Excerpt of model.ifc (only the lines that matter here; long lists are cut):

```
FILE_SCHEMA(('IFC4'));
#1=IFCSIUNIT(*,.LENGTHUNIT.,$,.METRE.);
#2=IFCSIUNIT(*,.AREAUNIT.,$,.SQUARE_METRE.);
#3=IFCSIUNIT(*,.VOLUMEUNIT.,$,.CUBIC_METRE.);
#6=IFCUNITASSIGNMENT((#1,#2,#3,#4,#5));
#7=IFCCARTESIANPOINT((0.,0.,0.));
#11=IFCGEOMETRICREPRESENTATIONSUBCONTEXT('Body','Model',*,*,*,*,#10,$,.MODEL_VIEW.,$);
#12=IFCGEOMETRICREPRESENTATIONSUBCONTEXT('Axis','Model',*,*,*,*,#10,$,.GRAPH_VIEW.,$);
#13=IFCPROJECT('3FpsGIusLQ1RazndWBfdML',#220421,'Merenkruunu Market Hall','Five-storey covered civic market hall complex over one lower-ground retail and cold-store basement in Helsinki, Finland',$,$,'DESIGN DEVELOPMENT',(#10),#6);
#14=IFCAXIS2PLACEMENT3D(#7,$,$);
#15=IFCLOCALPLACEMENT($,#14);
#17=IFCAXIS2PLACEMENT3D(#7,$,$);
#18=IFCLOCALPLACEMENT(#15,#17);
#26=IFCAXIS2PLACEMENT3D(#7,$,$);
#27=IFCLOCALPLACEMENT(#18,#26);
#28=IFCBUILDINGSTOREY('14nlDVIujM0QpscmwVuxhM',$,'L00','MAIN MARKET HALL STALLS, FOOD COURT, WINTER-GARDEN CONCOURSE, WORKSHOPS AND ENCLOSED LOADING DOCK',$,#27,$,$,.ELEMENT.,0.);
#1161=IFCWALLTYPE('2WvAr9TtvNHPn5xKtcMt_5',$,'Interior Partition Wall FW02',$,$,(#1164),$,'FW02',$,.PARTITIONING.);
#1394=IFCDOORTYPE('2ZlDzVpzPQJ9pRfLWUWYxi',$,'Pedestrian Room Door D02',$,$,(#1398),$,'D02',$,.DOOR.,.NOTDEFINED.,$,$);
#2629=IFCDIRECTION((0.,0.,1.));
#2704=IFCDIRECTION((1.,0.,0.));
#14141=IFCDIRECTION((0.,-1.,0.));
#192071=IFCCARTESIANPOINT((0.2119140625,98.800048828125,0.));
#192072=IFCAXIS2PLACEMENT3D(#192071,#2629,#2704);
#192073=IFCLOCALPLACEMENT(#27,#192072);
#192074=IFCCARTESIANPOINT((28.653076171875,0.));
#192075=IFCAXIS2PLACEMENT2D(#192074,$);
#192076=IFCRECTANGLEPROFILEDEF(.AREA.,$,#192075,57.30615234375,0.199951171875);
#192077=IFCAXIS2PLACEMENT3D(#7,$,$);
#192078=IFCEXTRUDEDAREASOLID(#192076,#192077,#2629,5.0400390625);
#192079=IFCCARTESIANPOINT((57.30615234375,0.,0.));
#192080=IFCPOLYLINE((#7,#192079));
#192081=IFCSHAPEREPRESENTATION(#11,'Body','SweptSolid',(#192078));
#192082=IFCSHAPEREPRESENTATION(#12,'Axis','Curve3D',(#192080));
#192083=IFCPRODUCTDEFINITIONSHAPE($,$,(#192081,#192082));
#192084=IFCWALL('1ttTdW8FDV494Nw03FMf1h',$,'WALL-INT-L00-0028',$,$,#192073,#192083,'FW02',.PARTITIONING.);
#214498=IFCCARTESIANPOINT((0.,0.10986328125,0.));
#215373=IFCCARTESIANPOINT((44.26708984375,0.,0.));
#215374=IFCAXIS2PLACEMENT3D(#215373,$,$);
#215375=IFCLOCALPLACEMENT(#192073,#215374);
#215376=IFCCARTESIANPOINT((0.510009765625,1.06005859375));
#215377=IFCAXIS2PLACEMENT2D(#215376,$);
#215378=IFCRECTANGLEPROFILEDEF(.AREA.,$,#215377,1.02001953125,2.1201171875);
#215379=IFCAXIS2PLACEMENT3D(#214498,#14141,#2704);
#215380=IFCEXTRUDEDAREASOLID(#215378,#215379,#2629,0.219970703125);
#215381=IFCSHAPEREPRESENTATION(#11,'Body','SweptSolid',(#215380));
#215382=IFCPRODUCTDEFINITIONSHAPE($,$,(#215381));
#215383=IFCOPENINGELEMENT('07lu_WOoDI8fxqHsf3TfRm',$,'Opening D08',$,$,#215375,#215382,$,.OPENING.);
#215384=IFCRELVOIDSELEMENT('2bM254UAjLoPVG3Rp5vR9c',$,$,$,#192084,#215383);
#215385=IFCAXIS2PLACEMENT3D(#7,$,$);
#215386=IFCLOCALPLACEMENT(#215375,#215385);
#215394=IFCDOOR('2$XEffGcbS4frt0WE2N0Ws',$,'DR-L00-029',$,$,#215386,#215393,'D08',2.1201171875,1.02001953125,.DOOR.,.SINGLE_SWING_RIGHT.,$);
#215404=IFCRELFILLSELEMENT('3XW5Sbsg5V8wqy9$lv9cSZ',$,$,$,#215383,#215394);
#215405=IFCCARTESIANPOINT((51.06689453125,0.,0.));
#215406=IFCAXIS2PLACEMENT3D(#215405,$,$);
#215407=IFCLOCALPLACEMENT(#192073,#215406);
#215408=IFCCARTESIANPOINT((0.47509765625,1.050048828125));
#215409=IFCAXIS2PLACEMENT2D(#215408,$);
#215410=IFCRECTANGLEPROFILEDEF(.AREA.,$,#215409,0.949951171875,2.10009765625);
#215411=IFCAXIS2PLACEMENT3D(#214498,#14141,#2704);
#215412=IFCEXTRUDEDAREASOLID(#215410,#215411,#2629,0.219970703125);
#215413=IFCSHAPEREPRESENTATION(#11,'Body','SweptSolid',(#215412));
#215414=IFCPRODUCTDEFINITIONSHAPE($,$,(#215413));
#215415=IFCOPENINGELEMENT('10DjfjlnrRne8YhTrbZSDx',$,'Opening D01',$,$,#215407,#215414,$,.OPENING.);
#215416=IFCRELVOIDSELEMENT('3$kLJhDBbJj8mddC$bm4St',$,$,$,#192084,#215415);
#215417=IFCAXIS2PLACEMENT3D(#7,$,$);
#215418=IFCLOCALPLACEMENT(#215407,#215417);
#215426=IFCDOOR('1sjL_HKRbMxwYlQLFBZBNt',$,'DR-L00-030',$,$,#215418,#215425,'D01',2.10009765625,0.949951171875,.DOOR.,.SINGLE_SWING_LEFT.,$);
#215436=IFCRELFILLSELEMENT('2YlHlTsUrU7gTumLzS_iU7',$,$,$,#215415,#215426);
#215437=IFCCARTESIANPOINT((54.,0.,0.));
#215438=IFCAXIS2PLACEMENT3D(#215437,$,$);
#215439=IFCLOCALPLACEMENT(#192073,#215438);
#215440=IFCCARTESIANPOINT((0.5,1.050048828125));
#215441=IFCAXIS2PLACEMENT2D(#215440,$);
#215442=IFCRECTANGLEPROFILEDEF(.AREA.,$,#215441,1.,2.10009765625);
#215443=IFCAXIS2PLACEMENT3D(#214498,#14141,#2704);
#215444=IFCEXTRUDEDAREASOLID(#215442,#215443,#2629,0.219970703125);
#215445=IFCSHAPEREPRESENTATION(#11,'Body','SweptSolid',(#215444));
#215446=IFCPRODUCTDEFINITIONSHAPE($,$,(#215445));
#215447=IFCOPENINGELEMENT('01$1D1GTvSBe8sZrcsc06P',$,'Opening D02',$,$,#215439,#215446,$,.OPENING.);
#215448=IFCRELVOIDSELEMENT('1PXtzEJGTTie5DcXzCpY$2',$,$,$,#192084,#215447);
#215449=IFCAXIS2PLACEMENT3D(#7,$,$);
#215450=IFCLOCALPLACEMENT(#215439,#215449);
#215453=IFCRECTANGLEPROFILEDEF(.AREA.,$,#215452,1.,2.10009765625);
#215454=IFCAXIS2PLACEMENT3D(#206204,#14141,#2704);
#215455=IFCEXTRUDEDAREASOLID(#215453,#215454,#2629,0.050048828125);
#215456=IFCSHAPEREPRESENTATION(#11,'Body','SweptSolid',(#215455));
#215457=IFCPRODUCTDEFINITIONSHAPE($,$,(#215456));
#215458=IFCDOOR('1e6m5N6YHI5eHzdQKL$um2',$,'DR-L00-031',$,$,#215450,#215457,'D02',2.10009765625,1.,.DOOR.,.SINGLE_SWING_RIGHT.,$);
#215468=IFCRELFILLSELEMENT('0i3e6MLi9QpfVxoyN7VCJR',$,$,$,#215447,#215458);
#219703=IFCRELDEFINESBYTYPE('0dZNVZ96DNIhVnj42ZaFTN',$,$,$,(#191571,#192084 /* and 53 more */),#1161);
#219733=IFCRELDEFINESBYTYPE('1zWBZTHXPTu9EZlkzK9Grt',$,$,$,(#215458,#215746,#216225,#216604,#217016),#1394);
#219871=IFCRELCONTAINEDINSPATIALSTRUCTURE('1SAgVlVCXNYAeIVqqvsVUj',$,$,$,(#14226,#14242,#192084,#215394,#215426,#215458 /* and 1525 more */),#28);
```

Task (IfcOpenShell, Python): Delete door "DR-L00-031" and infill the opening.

```python
import ifcopenshell
import ifcopenshell.api.feature
import ifcopenshell.api.root
import ifcopenshell.geom
import ifcopenshell.util.shape

model = ifcopenshell.open("model.ifc")
settings = ifcopenshell.geom.settings()


def volume(element):
    """Net volume in cubic metres, openings subtracted."""
    shape = ifcopenshell.geom.create_shape(settings, element)
    return ifcopenshell.util.shape.get_volume(shape.geometry)


door = model.by_guid("1e6m5N6YHI5eHzdQKL$um2")
opening = door.FillsVoids[0].RelatingOpeningElement
wall = opening.VoidsElements[0].RelatingBuildingElement
before = volume(wall)

ifcopenshell.api.root.remove_product(model, product=door)
ifcopenshell.api.feature.remove_feature(model, feature=opening)

after = volume(wall)

print(f"wall volume {before:.3f} -> {after:.3f} m3")

model.write("model_updated.ifc")
```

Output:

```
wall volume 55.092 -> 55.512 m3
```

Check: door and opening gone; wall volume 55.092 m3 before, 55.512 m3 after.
